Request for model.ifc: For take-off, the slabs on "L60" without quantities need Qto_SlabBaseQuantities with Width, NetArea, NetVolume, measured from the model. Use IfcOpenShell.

First a look at what the model holds.

```python
import ifcopenshell
import ifcopenshell.util.element
import ifcopenshell.util.unit

model = ifcopenshell.open("model.ifc")
print(model.schema)
for unit_type in ("LENGTHUNIT", "AREAUNIT", "VOLUMEUNIT"):
    print(unit_type, ifcopenshell.util.unit.calculate_unit_scale(model, unit_type))
storey = next(s for s in model.by_type("IfcBuildingStorey") if s.Name == "L60")
slabs = [e for e in ifcopenshell.util.element.get_decomposition(storey) if e.is_a("IfcSlab")]
for e in sorted(slabs, key=lambda e: e.id()):
    print(e.id(), e.is_a(), e.Name, list(ifcopenshell.util.element.get_psets(e, qtos_only=True)), sep=" | ")
```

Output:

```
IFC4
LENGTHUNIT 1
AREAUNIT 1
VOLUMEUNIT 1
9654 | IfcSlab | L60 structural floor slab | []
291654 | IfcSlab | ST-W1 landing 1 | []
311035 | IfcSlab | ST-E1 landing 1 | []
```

```python
import ifcopenshell
import ifcopenshell.api.pset
import ifcopenshell.geom
import ifcopenshell.util.element
import ifcopenshell.util.shape
import ifcopenshell.util.unit

model = ifcopenshell.open("model.ifc")
unit_scale = ifcopenshell.util.unit.calculate_unit_scale(model)
area_scale = ifcopenshell.util.unit.calculate_unit_scale(model, "AREAUNIT")
volume_scale = ifcopenshell.util.unit.calculate_unit_scale(model, "VOLUMEUNIT")
settings = ifcopenshell.geom.settings()

storey = next(s for s in model.by_type("IfcBuildingStorey") if s.Name == "L60")
slabs = [e for e in ifcopenshell.util.element.get_decomposition(storey) if e.is_a("IfcSlab")]

for e in sorted(slabs, key=lambda e: e.id()):
    if ifcopenshell.util.element.get_psets(e, qtos_only=True, should_inherit=False):
        continue
    # Geometry comes back in metres, in the element's own axes.
    shape = ifcopenshell.geom.create_shape(settings, e)
    values = {
        "Width": ifcopenshell.util.shape.get_z(shape.geometry) / unit_scale,
        "NetArea": ifcopenshell.util.shape.get_footprint_area(shape.geometry) / area_scale,
        "NetVolume": ifcopenshell.util.shape.get_volume(shape.geometry) / volume_scale,
    }
    qto = ifcopenshell.api.pset.add_qto(model, product=e, name="Qto_SlabBaseQuantities")
    ifcopenshell.api.pset.edit_qto(model, qto=qto, properties=values)
    print(e.id(), {k: round(v, 3) for k, v in values.items()})

model.write("model_edited.ifc")
```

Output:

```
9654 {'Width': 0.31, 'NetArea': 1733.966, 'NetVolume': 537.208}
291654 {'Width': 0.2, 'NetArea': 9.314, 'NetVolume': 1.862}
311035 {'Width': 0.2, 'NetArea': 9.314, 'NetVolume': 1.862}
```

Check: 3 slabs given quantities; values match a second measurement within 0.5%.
